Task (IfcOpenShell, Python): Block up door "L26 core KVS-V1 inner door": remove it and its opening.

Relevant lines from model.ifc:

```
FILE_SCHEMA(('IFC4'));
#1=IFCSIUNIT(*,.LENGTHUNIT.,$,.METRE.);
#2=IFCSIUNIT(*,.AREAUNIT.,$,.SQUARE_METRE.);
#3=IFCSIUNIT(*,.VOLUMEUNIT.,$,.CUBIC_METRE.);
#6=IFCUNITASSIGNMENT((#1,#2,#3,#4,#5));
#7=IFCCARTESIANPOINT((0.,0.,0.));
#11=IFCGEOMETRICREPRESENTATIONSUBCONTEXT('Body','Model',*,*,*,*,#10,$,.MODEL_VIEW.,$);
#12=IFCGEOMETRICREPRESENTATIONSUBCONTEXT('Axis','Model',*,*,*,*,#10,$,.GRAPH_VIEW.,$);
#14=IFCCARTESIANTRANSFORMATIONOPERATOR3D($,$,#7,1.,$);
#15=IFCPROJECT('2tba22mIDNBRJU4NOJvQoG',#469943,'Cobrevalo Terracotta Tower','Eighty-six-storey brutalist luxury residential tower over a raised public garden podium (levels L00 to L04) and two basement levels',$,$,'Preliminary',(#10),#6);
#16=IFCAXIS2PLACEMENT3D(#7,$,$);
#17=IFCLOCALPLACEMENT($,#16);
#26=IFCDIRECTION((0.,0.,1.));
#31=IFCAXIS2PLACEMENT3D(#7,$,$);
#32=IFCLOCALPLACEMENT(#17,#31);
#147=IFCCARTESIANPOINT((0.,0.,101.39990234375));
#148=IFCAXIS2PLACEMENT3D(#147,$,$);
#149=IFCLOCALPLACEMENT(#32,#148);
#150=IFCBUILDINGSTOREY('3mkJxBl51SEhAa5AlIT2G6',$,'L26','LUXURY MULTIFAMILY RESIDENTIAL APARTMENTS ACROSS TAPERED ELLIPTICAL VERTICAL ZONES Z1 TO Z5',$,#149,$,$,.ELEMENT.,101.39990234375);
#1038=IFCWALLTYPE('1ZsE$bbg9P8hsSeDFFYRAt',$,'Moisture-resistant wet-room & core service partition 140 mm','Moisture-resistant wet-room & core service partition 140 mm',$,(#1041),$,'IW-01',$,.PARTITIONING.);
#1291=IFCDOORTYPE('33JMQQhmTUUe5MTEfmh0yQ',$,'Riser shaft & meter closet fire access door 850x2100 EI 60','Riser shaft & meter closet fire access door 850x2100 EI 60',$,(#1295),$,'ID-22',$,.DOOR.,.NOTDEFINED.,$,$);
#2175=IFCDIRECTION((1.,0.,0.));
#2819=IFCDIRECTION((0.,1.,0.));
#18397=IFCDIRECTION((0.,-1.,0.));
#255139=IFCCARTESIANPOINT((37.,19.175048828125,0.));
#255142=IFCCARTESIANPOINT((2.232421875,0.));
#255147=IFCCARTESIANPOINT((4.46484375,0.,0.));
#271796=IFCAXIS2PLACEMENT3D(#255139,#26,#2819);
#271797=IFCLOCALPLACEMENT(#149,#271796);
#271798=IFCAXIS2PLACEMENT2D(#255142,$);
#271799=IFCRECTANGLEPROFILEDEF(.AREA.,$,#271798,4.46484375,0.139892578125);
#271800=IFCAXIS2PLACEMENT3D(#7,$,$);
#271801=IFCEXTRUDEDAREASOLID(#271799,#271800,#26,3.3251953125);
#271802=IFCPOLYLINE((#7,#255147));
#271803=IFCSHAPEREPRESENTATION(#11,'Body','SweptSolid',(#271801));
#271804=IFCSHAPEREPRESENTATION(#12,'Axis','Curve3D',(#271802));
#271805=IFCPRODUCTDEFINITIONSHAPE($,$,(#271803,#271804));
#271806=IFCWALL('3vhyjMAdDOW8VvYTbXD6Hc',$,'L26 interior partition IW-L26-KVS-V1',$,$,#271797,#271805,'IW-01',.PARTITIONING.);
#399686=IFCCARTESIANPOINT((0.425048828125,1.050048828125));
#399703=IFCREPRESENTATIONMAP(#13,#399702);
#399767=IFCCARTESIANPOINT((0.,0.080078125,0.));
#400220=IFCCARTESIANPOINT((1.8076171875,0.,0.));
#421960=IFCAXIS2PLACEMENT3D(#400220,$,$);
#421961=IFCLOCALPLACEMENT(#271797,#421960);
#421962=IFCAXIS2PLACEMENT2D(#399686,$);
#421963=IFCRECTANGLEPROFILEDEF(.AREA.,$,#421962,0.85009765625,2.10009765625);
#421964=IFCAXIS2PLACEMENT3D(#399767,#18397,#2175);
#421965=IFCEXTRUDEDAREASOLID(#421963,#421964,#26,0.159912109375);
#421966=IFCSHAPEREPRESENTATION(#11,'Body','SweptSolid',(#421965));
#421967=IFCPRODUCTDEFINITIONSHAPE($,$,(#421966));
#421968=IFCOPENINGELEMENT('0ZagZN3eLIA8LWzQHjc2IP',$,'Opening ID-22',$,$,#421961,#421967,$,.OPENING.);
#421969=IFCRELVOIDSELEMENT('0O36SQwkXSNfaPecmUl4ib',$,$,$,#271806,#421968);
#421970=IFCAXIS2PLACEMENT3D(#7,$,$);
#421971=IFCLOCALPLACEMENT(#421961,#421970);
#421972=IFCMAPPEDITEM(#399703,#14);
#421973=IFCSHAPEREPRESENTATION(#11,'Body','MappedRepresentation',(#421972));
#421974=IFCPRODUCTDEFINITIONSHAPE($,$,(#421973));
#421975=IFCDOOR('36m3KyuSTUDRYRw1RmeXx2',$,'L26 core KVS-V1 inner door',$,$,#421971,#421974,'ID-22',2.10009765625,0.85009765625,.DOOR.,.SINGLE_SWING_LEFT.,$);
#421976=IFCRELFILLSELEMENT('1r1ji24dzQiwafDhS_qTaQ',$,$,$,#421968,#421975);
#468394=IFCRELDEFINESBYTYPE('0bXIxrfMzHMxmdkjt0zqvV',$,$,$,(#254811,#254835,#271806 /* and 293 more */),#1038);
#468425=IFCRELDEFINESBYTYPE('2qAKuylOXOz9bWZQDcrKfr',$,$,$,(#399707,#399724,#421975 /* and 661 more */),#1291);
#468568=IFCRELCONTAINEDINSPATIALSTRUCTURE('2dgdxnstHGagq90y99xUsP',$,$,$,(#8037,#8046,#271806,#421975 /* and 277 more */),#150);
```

```python
import ifcopenshell
import ifcopenshell.api.feature
import ifcopenshell.api.root
import ifcopenshell.geom
import ifcopenshell.util.shape

model = ifcopenshell.open("model.ifc")
settings = ifcopenshell.geom.settings()


def volume(element):
    """Net volume in cubic metres, openings subtracted."""
    shape = ifcopenshell.geom.create_shape(settings, element)
    return ifcopenshell.util.shape.get_volume(shape.geometry)


door = model.by_guid("36m3KyuSTUDRYRw1RmeXx2")
opening = door.FillsVoids[0].RelatingOpeningElement
wall = opening.VoidsElements[0].RelatingBuildingElement
before = volume(wall)

ifcopenshell.api.root.remove_product(model, product=door)
ifcopenshell.api.feature.remove_feature(model, feature=opening)

after = volume(wall)

print(f"wall volume {before:.3f} -> {after:.3f} m3")

model.write("model_updated.ifc")
```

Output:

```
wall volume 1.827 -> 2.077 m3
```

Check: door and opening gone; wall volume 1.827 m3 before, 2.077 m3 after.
